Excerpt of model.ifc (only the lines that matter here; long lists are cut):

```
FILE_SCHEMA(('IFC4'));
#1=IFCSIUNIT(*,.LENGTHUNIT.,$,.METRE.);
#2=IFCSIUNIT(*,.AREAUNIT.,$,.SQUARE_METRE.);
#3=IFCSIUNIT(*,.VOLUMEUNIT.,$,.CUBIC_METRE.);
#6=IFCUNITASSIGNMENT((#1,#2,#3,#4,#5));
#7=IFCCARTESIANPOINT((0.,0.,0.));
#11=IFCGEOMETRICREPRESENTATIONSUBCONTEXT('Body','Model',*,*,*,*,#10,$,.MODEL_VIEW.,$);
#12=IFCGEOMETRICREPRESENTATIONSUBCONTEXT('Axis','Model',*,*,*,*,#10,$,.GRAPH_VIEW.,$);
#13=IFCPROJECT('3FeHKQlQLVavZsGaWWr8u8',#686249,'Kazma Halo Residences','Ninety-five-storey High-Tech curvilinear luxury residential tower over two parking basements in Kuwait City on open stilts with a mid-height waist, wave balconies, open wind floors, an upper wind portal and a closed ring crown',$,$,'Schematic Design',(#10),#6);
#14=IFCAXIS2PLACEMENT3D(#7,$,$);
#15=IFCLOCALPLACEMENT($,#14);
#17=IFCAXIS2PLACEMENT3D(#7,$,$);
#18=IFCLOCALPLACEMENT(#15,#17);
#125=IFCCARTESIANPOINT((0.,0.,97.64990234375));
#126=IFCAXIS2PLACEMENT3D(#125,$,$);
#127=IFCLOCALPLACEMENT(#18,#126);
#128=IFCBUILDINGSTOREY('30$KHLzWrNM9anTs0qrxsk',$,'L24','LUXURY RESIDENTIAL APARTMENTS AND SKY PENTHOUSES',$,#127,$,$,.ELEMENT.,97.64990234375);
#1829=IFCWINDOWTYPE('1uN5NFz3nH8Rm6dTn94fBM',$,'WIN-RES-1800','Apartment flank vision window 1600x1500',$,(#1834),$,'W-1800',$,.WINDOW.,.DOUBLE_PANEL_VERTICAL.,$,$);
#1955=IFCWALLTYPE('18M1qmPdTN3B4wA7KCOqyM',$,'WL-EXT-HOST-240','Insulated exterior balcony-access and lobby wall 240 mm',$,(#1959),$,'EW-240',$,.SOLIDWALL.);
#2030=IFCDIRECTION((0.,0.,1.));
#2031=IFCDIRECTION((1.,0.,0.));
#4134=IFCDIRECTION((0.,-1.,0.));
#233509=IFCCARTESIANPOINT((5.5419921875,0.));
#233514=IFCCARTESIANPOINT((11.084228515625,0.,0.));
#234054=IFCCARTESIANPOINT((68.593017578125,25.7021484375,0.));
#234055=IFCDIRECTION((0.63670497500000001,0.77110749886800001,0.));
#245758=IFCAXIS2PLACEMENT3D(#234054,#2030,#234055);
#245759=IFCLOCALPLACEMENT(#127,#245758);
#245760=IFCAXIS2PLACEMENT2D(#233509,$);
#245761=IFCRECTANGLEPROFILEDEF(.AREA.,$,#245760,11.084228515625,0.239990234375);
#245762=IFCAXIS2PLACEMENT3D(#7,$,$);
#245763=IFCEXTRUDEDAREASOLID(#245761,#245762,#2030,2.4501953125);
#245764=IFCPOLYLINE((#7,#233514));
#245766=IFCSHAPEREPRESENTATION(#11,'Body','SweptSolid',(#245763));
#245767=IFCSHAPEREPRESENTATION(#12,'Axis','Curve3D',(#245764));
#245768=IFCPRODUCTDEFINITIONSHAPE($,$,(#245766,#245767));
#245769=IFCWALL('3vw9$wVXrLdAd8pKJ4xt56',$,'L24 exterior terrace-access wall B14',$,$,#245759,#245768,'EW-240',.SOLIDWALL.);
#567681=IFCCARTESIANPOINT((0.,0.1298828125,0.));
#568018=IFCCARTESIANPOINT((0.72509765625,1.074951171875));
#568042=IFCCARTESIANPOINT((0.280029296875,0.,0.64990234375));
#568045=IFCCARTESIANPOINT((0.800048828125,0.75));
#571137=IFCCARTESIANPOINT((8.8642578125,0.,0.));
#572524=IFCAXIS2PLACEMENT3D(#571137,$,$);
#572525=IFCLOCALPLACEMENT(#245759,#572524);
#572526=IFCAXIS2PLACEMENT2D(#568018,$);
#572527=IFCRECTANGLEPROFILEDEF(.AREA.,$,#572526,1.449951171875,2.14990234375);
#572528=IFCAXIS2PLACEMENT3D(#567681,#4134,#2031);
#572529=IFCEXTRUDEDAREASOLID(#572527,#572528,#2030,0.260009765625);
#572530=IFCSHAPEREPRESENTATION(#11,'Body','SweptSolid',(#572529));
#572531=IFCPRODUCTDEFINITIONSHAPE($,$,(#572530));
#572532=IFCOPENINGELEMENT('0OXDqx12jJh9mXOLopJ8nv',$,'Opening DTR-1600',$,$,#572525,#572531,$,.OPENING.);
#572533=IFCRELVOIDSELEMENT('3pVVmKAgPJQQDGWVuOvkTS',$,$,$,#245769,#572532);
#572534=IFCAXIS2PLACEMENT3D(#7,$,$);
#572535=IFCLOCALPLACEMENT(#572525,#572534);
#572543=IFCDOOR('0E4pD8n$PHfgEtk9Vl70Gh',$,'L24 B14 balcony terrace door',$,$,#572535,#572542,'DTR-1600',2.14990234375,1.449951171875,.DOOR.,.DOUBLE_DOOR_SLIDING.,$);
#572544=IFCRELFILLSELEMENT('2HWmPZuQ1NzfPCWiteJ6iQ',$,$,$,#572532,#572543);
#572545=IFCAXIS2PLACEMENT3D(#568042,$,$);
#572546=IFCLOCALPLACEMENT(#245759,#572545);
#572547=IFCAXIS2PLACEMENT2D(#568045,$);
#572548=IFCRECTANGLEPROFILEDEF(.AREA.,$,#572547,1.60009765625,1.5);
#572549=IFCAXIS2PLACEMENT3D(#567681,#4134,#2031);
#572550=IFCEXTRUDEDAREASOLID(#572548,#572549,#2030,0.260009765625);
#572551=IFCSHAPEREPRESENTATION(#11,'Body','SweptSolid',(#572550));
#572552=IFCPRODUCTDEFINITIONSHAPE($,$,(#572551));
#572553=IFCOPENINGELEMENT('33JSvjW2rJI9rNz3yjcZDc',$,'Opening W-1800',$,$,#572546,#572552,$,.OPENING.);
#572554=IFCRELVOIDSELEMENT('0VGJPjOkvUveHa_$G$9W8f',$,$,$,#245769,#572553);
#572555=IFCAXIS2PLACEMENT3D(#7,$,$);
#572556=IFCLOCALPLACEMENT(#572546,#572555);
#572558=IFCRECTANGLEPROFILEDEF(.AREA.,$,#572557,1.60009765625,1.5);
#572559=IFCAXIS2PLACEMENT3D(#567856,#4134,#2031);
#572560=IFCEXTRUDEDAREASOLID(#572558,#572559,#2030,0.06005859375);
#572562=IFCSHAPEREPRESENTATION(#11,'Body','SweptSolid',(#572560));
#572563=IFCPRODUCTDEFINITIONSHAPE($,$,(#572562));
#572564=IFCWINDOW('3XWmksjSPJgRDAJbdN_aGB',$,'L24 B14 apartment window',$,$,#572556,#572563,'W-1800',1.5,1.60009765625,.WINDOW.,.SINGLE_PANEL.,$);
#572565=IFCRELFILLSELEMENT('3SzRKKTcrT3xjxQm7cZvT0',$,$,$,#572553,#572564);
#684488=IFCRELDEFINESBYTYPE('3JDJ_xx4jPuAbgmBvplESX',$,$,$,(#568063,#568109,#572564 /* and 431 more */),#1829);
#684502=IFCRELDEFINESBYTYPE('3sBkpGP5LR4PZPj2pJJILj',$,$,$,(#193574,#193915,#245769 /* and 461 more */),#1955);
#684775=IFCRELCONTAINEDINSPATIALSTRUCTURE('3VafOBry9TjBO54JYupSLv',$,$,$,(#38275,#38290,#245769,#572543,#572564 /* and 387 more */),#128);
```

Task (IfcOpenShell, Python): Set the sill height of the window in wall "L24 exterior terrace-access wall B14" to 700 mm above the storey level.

```python
import numpy as np
import ifcopenshell
import ifcopenshell.api.geometry
import ifcopenshell.geom
import ifcopenshell.util.element
import ifcopenshell.util.placement
import ifcopenshell.util.shape
import ifcopenshell.util.unit

model = ifcopenshell.open("model.ifc")
unit_scale = ifcopenshell.util.unit.calculate_unit_scale(model)

window = model.by_guid("3XWmksjSPJgRDAJbdN_aGB")
opening = window.FillsVoids[0].RelatingOpeningElement
storey = ifcopenshell.util.element.get_container(window, ifc_class="IfcBuildingStorey")
level = ifcopenshell.util.placement.get_local_placement(storey.ObjectPlacement)[2, 3]

# The opening's origin need not be at the sill, so measure its lowest point.
shape = ifcopenshell.geom.create_shape(ifcopenshell.geom.settings(), opening)
bottom = ifcopenshell.util.shape.get_shape_bottom_elevation(shape, shape.geometry) / unit_scale
dz = level + 0.7 / unit_scale - bottom

shift = np.array([0.0, 0.0, dz])
# The window is placed relative to its opening, so it follows when the opening moves.
matrix = ifcopenshell.util.placement.get_local_placement(opening.ObjectPlacement)
matrix[:3, 3] += shift
ifcopenshell.api.geometry.edit_object_placement(
    model, product=opening, matrix=matrix, is_si=False, should_transform_children=True
)

print(f"moved by {dz * unit_scale:+.3f} m")

model.write("model-out.ifc")
```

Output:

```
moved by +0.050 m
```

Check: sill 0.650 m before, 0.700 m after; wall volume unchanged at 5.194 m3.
